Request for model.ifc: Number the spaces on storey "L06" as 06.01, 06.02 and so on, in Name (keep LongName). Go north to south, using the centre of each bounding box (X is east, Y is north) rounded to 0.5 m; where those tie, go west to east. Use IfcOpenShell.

First a look at what the model holds.

```python
import ifcopenshell
import ifcopenshell.util.element
import ifcopenshell.util.placement

model = ifcopenshell.open("model.ifc")
print(model.schema)
storey = next(s for s in model.by_type("IfcBuildingStorey") if s.Name == "L06")
spaces = [e for e in ifcopenshell.util.element.get_decomposition(storey) if e.is_a("IfcSpace")]
for e in sorted(spaces, key=lambda e: e.id()):
    origin = ifcopenshell.util.placement.get_local_placement(e.ObjectPlacement)[:3, 3]
    print(e.id(), e.Name, e.LongName, origin.round(2) + 0.0, sep=" | ")
```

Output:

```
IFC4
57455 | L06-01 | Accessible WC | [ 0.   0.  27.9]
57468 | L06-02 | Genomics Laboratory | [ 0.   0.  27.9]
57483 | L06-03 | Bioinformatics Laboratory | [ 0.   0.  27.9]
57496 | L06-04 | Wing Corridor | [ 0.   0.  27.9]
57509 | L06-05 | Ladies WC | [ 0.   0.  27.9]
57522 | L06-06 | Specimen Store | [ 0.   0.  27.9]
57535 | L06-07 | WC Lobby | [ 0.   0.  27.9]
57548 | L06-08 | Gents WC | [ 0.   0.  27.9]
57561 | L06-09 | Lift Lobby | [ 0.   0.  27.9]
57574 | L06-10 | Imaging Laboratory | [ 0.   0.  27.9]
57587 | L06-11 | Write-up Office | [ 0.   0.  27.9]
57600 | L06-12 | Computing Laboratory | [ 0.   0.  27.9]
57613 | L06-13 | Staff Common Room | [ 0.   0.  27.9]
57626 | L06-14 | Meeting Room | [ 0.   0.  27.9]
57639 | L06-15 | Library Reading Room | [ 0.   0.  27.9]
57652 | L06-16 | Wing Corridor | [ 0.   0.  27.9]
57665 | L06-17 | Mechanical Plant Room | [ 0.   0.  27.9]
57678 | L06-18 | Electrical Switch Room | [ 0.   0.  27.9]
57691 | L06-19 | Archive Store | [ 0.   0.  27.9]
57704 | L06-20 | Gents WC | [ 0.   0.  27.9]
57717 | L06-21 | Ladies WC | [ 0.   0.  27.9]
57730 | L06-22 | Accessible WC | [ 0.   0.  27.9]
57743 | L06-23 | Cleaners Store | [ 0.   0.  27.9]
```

```python
import ifcopenshell
import ifcopenshell.geom
import ifcopenshell.util.element
import ifcopenshell.util.shape

model = ifcopenshell.open("model.ifc")
settings = ifcopenshell.geom.settings()
settings.set("use-world-coords", True)


def centre(element):
    shape = ifcopenshell.geom.create_shape(settings, element)
    return ifcopenshell.util.shape.get_bbox_centroid(shape.geometry)


storey = next(s for s in model.by_type("IfcBuildingStorey") if s.Name == "L06")
spaces = [e for e in ifcopenshell.util.element.get_decomposition(storey) if e.is_a("IfcSpace")]

# Insertion points can sit at a corner or the storey origin, so sort by the geometry (in metres).
centres = {e: centre(e) for e in spaces}
spaces.sort(key=lambda e: (-round(centres[e][1] / 0.5), centres[e][0]))

for i, e in enumerate(spaces, start=1):
    number = f"06.{i:02d}"
    e.Name = number
    print(e.id(), number)

model.write("model_v2.ifc")
```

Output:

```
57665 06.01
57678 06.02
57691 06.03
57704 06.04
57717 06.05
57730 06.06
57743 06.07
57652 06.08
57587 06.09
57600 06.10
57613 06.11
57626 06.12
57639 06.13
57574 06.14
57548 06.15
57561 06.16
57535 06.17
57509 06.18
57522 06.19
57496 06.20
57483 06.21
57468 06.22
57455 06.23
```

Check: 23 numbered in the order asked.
